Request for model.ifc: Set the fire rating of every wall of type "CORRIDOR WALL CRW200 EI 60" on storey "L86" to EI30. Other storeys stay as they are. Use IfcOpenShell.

First a look at what the model holds.

```python
import ifcopenshell
import ifcopenshell.util.element

model = ifcopenshell.open("model.ifc")
print(model.schema)
storey = next(s for s in model.by_type("IfcBuildingStorey") if s.Name == "L86")
walls = [e for e in ifcopenshell.util.element.get_decomposition(storey) if e.is_a("IfcWall")]
seen = {}
for e in walls:
    element_type = ifcopenshell.util.element.get_type(e)
    key = (element_type.Name if element_type != e and element_type else None, ifcopenshell.util.element.get_pset(e, "Pset_WallCommon", "FireRating"))
    seen[key] = seen.get(key, 0) + 1
for (name, value), count in sorted(seen.items(), key=str):
    print(count, "x", name, "|", value)
```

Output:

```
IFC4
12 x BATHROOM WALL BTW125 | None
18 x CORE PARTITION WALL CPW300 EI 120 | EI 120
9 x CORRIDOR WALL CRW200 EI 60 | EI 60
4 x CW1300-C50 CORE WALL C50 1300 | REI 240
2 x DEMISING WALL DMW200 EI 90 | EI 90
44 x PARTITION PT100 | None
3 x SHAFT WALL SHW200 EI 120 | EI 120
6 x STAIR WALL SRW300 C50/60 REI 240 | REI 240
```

```python
import ifcopenshell
import ifcopenshell.api.pset
import ifcopenshell.util.element

model = ifcopenshell.open("model.ifc")

storey = next(s for s in model.by_type("IfcBuildingStorey") if s.Name == "L86")
walls = [e for e in ifcopenshell.util.element.get_decomposition(storey) if e.is_a("IfcWall")]

count = 0
for e in walls:
    element_type = ifcopenshell.util.element.get_type(e)
    if element_type in (None, e) or element_type.Name != "CORRIDOR WALL CRW200 EI 60":
        continue
    found = ifcopenshell.util.element.get_pset(e, "Pset_WallCommon", should_inherit=False)
    if found:
        pset = model.by_id(found["id"])
        if len(ifcopenshell.util.element.get_elements_by_pset(pset)) > 1:
            pset = ifcopenshell.api.pset.unshare_pset(model, products=[e], pset=pset)[0]
    else:
        pset = ifcopenshell.api.pset.add_pset(model, product=e, name="Pset_WallCommon")
    ifcopenshell.api.pset.edit_pset(model, pset=pset, properties={"FireRating": "EI30"})
    count += 1

print(count, "walls updated")

model.write("model_edited.ifc")
```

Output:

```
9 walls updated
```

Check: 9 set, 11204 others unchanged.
